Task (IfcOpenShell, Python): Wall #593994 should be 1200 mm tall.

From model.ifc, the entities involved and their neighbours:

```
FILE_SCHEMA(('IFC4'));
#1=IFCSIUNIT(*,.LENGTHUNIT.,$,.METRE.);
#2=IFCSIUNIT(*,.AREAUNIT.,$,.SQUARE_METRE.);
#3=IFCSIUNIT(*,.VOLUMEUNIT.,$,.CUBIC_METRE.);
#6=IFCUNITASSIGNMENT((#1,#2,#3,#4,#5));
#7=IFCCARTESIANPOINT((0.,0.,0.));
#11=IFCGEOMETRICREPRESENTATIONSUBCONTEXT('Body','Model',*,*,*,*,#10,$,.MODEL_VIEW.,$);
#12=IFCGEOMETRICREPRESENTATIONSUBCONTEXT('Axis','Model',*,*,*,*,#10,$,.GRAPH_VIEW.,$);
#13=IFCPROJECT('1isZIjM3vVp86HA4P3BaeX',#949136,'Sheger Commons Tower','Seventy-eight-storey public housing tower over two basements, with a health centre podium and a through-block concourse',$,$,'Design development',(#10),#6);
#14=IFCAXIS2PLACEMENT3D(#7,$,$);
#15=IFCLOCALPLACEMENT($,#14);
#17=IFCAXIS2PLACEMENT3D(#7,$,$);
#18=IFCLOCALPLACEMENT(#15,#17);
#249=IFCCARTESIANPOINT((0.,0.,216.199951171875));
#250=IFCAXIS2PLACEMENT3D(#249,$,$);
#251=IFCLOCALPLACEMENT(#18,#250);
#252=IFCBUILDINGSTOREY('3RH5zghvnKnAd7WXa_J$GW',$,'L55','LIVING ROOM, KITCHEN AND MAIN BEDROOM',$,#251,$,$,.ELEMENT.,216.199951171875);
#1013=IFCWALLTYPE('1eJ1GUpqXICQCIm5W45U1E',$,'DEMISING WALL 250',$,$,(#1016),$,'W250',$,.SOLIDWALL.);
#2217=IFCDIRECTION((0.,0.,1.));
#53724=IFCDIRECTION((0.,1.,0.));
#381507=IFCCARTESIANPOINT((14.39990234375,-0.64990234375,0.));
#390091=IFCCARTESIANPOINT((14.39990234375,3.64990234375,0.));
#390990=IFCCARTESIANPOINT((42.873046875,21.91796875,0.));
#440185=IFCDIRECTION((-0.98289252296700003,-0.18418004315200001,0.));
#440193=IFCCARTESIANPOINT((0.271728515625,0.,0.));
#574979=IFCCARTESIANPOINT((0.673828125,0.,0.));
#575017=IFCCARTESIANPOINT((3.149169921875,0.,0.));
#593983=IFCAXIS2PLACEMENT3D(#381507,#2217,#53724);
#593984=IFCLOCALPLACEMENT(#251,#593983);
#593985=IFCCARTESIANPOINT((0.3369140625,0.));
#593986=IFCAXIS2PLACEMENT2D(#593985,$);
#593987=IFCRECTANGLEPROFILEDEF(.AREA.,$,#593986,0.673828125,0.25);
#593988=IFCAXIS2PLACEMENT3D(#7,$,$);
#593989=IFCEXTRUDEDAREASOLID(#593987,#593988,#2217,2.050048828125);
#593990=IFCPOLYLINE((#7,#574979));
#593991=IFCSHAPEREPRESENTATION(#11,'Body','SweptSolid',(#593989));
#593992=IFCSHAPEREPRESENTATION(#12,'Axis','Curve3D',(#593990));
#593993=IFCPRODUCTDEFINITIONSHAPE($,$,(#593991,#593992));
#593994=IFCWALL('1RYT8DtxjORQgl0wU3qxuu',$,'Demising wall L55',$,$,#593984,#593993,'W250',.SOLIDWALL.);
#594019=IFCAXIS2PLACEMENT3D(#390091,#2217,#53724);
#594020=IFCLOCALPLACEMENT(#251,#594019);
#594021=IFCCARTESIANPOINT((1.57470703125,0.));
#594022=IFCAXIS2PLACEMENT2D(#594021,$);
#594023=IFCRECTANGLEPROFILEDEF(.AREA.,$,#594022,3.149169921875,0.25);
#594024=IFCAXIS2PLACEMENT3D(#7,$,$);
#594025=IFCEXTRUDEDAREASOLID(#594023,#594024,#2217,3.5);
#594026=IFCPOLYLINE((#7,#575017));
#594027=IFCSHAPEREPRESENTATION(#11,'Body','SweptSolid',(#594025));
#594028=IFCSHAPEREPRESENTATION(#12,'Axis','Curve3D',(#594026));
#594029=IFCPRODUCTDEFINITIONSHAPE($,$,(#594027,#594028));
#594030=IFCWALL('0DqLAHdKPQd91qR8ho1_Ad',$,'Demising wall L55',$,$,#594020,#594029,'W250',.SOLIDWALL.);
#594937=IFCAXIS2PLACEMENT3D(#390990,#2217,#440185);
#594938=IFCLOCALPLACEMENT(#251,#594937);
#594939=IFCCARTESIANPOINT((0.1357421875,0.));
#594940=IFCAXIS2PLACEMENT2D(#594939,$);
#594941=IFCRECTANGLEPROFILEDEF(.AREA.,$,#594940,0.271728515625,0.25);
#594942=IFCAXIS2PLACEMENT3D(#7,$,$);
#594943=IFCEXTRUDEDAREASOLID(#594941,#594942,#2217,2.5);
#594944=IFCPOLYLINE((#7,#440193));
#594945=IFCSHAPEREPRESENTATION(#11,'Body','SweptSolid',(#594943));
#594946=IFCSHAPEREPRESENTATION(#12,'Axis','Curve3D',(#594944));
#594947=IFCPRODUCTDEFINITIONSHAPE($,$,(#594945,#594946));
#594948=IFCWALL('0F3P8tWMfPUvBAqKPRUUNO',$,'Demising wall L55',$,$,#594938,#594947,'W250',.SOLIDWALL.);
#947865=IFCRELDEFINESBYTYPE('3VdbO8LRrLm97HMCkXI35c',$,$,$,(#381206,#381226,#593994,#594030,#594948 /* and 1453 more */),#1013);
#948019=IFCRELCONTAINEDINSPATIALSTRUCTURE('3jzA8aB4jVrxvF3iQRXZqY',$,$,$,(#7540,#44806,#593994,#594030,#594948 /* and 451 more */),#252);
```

```python
import ifcopenshell
import ifcopenshell.geom
import ifcopenshell.util.representation
import ifcopenshell.util.shape
import ifcopenshell.util.unit

model = ifcopenshell.open("model.ifc")
unit_scale = ifcopenshell.util.unit.calculate_unit_scale(model)
settings = ifcopenshell.geom.settings()


def volume(element):
    """Net volume in cubic metres, openings subtracted."""
    shape = ifcopenshell.geom.create_shape(settings, element)
    return ifcopenshell.util.shape.get_volume(shape.geometry)


wall = model.by_id(593994)
before = volume(wall)

body = ifcopenshell.util.representation.get_representation(wall, "Model", "Body")
solid = body.Items[0]
old_height = solid.Depth
solid.Depth = 1.2 / unit_scale
after = volume(wall)

print(f"height {old_height:g} -> {solid.Depth:g}, volume {before:.3f} -> {after:.3f} m3")

model.write("model-out.ifc")
```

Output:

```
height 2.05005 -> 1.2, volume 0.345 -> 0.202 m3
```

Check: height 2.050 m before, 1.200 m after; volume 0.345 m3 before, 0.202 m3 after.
